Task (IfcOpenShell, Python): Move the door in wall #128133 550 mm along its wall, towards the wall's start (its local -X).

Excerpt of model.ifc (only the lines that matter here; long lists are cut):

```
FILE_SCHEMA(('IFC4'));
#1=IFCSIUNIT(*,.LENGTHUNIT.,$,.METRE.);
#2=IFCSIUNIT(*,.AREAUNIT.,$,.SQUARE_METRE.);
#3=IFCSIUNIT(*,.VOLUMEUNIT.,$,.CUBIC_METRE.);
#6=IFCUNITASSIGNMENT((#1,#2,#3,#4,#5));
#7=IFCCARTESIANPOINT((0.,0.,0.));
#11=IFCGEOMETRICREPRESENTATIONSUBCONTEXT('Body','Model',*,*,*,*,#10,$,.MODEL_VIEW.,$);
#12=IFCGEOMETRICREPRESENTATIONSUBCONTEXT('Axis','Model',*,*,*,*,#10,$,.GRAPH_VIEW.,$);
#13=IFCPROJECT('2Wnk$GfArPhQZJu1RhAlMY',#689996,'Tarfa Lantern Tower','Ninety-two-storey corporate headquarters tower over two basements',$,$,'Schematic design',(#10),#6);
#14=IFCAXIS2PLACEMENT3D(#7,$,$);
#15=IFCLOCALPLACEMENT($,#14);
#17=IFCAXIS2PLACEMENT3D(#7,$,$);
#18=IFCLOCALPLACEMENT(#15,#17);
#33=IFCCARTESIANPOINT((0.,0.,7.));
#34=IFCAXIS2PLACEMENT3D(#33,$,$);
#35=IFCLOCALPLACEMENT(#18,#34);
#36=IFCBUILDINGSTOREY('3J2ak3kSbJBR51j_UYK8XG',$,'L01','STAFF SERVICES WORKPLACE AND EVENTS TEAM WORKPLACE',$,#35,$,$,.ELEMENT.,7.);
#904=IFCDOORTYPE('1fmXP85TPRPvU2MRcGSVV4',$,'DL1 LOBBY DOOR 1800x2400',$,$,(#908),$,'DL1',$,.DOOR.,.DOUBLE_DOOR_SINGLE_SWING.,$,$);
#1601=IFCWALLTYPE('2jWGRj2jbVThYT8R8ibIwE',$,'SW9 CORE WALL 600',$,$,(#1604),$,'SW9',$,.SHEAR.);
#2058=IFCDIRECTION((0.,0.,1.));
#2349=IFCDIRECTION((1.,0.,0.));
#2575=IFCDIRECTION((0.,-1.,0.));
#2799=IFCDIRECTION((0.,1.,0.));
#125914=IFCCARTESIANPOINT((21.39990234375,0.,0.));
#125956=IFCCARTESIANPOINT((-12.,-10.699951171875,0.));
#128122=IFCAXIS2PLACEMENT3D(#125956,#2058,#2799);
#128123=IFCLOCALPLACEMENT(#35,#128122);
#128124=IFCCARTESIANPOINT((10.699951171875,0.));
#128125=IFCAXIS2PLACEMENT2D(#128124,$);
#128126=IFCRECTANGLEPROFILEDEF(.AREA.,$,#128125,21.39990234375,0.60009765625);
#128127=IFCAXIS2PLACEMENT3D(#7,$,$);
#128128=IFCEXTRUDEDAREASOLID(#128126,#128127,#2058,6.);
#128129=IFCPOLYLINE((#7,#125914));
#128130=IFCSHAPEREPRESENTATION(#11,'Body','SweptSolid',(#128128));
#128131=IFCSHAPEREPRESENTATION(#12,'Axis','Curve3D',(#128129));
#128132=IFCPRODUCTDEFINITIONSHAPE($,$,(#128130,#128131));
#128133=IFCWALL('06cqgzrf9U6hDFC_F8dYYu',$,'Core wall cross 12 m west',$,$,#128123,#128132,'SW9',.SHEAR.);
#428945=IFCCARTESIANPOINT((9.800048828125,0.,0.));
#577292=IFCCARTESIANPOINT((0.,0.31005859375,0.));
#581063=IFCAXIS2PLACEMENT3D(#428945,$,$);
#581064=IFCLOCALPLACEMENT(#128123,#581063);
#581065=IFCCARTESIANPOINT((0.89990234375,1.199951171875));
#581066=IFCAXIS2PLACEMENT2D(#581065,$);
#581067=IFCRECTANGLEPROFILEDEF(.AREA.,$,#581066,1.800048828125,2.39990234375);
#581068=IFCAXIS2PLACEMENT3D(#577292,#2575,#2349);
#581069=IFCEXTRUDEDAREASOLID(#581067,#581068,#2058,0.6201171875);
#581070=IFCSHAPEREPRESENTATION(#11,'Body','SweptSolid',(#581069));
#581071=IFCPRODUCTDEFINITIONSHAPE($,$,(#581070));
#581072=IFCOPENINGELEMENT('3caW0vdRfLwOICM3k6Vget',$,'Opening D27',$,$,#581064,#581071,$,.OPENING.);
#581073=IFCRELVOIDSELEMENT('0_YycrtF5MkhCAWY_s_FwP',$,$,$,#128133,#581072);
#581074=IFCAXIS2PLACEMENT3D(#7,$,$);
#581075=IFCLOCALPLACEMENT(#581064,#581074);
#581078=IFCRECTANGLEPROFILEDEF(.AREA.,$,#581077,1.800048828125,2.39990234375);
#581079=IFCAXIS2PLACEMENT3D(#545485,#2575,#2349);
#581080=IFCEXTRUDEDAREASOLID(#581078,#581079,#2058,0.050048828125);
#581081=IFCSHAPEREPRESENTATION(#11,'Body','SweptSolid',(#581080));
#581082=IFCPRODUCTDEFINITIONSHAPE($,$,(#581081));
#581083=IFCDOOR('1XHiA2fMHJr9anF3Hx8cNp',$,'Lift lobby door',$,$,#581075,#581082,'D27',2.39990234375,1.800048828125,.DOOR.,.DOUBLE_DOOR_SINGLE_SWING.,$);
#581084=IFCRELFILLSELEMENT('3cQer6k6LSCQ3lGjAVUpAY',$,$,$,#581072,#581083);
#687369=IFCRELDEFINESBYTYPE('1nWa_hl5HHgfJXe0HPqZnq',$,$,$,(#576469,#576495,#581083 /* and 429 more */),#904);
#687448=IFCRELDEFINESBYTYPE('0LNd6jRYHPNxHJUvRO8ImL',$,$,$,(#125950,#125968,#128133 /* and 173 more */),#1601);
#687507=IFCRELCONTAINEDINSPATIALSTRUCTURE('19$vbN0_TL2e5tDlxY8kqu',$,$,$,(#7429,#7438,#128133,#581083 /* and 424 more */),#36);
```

```python
import ifcopenshell
import ifcopenshell.api.geometry
import ifcopenshell.util.placement
import ifcopenshell.util.unit

model = ifcopenshell.open("model.ifc")
unit_scale = ifcopenshell.util.unit.calculate_unit_scale(model)

door = model.by_guid("1XHiA2fMHJr9anF3Hx8cNp")
opening = door.FillsVoids[0].RelatingOpeningElement
wall = opening.VoidsElements[0].RelatingBuildingElement

wall_matrix = ifcopenshell.util.placement.get_local_placement(wall.ObjectPlacement)
shift = wall_matrix[:3, 0] * -0.55 / unit_scale
before = ifcopenshell.util.placement.get_local_placement(door.ObjectPlacement)[:3, 3].copy()

# The door is placed relative to its opening, so it follows when the opening moves.
matrix = ifcopenshell.util.placement.get_local_placement(opening.ObjectPlacement)
matrix[:3, 3] += shift
ifcopenshell.api.geometry.edit_object_placement(
    model, product=opening, matrix=matrix, is_si=False, should_transform_children=True
)

after = ifcopenshell.util.placement.get_local_placement(door.ObjectPlacement)[:3, 3]
print("door moved by", (after - before).round(3) + 0.0)

model.write("model_edited.ifc")
```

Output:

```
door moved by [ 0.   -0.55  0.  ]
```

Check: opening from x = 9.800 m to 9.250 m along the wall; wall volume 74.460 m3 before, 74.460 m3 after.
